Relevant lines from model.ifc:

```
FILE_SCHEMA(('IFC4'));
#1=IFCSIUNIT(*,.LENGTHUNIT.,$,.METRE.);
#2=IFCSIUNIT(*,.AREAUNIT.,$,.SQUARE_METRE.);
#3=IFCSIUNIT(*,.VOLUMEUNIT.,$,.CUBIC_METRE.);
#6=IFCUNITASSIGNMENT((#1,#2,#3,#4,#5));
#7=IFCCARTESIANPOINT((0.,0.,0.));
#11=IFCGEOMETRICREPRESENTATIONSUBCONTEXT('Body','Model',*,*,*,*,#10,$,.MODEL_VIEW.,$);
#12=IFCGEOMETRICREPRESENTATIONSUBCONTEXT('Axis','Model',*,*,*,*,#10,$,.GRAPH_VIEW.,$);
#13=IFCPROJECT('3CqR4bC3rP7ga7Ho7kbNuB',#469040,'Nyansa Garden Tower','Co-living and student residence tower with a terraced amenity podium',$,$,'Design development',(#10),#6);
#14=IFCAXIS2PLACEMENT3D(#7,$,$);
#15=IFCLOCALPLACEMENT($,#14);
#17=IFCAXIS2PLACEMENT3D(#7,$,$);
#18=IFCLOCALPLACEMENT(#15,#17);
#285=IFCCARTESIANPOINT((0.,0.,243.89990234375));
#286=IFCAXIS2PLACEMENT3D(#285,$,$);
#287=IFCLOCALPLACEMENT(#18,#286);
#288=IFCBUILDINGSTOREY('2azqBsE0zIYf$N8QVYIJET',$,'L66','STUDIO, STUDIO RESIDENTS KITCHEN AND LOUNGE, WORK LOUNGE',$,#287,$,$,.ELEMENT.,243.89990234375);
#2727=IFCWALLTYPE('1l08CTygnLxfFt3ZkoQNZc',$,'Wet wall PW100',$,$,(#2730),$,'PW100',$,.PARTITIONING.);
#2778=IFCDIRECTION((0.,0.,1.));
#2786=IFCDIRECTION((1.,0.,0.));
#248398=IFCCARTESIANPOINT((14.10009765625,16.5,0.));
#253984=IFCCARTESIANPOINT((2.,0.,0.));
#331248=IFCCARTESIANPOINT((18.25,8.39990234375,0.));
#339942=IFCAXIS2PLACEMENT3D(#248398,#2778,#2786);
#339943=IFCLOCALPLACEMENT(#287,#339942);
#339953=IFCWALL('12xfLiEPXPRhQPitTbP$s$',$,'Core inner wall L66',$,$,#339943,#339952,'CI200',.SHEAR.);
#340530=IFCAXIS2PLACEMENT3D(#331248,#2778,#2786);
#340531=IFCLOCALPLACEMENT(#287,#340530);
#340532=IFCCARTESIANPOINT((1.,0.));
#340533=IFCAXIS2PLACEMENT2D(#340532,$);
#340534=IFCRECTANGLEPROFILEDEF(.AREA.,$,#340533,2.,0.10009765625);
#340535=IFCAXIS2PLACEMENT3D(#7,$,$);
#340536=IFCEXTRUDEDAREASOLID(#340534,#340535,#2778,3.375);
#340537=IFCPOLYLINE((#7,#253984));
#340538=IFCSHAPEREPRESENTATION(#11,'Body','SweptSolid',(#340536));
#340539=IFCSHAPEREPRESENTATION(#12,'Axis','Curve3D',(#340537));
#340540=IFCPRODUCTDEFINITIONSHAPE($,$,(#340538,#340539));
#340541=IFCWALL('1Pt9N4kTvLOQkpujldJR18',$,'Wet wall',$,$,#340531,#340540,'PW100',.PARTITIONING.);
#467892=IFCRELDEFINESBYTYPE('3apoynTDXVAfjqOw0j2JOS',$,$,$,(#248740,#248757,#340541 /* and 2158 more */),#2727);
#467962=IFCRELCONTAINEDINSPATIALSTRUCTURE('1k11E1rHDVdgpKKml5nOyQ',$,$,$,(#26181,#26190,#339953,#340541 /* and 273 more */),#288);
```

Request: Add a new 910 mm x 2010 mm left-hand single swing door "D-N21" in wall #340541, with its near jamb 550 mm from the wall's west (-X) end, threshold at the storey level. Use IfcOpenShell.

```python
import numpy as np
import ifcopenshell
import ifcopenshell.api.feature
import ifcopenshell.api.geometry
import ifcopenshell.api.root
import ifcopenshell.api.spatial
import ifcopenshell.geom
import ifcopenshell.util.element
import ifcopenshell.util.placement
import ifcopenshell.util.representation
import ifcopenshell.util.shape
import ifcopenshell.util.unit

model = ifcopenshell.open("model.ifc")
unit_scale = ifcopenshell.util.unit.calculate_unit_scale(model)
settings = ifcopenshell.geom.settings()


def volume(element):
    """Net volume in cubic metres, openings subtracted."""
    shape = ifcopenshell.geom.create_shape(settings, element)
    return ifcopenshell.util.shape.get_volume(shape.geometry)


wall = model.by_id(340541)
storey = ifcopenshell.util.element.get_container(wall, ifc_class="IfcBuildingStorey")
context = ifcopenshell.util.representation.get_context(model, "Model", "Body", "MODEL_VIEW")
before = volume(wall)

width, height, from_end, sill = 0.91, 2.01, 0.55, 0.0  # metres

# The wall runs along its own X axis, and the end named is its -X end.
wall_shape = ifcopenshell.geom.create_shape(settings, wall)
x, y, z = ifcopenshell.util.shape.get_vertices(wall_shape.geometry).T
start = x.min() + from_end
face, thickness = float(y.min()), float(y.max() - y.min())
wall_matrix = ifcopenshell.util.placement.get_local_placement(wall.ObjectPlacement)
level = ifcopenshell.util.placement.get_local_placement(storey.ObjectPlacement)[2, 3]


def in_wall(x, y):
    """Placement at x, y metres in the wall's axes, at sill height."""
    matrix = wall_matrix.copy()
    matrix[:, 3] = wall_matrix @ np.array([x / unit_scale, y / unit_scale, 0.0, 1.0])
    matrix[2, 3] = level + sill / unit_scale
    return matrix


# Opening: a box that overshoots both wall faces by 50 mm.
opening = ifcopenshell.api.root.create_entity(model, ifc_class="IfcOpeningElement", predefined_type="OPENING")
box = ifcopenshell.api.geometry.add_wall_representation(
    model, context=context, length=width, height=height, thickness=thickness + 0.1
)
ifcopenshell.api.geometry.assign_representation(model, product=opening, representation=box)
ifcopenshell.api.geometry.edit_object_placement(model, product=opening, matrix=in_wall(start, face - 0.05), is_si=False)
ifcopenshell.api.feature.add_feature(model, feature=opening, element=wall)

door = ifcopenshell.api.root.create_entity(model, ifc_class="IfcDoor", name="D-N21", predefined_type="DOOR")
door.OverallWidth, door.OverallHeight = width / unit_scale, height / unit_scale
door.OperationType = "SINGLE_SWING_LEFT"
body = ifcopenshell.api.geometry.add_door_representation(
    model,
    context=context,
    overall_width=door.OverallWidth,
    overall_height=door.OverallHeight,
    operation_type="SINGLE_SWING_LEFT",
    lining_properties={"LiningDepth": thickness / unit_scale, "ThresholdDepth": thickness / unit_scale},
)
ifcopenshell.api.geometry.assign_representation(model, product=door, representation=body)
ifcopenshell.api.spatial.assign_container(model, products=[door], relating_structure=storey)
ifcopenshell.api.feature.add_filling(model, opening=opening, element=door)

# The lining spans the wall, so the door starts at the wall face.
ifcopenshell.api.geometry.edit_object_placement(model, product=door, matrix=in_wall(start, face), is_si=False)

after = volume(wall)

print(f"wall volume {before:.3f} -> {after:.3f} m3")

model.write("model_rev.ifc")
```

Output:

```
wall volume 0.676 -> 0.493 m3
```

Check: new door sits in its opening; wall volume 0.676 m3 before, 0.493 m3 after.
